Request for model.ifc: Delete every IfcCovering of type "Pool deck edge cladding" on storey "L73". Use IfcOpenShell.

First a look at what the model holds.

```python
import ifcopenshell
import ifcopenshell.util.element

model = ifcopenshell.open("model.ifc")
print(model.schema)
storey = next(s for s in model.by_type("IfcBuildingStorey") if s.Name == "L73")
coverings = [e for e in ifcopenshell.util.element.get_decomposition(storey) if e.is_a("IfcCovering")]
seen = {}
for e in coverings:
    element_type = ifcopenshell.util.element.get_type(e)
    name = element_type.Name if element_type not in (None, e) else None
    seen[name] = seen.get(name, 0) + 1
for name, count in sorted(seen.items(), key=str):
    print(count, "x", name)
```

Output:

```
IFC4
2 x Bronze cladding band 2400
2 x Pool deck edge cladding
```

```python
import ifcopenshell
import ifcopenshell.api.root
import ifcopenshell.util.element

model = ifcopenshell.open("model.ifc")

storey = next(s for s in model.by_type("IfcBuildingStorey") if s.Name == "L73")
coverings = [e for e in ifcopenshell.util.element.get_decomposition(storey) if e.is_a("IfcCovering")]
targets = [e for e in coverings if (t := ifcopenshell.util.element.get_type(e)) not in (None, e) and t.Name == "Pool deck edge cladding"]

for e in targets:
    ifcopenshell.api.root.remove_product(model, product=e)
print(len(targets), "removed")

model.write("model_edited.ifc")
```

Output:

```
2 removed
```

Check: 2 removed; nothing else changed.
